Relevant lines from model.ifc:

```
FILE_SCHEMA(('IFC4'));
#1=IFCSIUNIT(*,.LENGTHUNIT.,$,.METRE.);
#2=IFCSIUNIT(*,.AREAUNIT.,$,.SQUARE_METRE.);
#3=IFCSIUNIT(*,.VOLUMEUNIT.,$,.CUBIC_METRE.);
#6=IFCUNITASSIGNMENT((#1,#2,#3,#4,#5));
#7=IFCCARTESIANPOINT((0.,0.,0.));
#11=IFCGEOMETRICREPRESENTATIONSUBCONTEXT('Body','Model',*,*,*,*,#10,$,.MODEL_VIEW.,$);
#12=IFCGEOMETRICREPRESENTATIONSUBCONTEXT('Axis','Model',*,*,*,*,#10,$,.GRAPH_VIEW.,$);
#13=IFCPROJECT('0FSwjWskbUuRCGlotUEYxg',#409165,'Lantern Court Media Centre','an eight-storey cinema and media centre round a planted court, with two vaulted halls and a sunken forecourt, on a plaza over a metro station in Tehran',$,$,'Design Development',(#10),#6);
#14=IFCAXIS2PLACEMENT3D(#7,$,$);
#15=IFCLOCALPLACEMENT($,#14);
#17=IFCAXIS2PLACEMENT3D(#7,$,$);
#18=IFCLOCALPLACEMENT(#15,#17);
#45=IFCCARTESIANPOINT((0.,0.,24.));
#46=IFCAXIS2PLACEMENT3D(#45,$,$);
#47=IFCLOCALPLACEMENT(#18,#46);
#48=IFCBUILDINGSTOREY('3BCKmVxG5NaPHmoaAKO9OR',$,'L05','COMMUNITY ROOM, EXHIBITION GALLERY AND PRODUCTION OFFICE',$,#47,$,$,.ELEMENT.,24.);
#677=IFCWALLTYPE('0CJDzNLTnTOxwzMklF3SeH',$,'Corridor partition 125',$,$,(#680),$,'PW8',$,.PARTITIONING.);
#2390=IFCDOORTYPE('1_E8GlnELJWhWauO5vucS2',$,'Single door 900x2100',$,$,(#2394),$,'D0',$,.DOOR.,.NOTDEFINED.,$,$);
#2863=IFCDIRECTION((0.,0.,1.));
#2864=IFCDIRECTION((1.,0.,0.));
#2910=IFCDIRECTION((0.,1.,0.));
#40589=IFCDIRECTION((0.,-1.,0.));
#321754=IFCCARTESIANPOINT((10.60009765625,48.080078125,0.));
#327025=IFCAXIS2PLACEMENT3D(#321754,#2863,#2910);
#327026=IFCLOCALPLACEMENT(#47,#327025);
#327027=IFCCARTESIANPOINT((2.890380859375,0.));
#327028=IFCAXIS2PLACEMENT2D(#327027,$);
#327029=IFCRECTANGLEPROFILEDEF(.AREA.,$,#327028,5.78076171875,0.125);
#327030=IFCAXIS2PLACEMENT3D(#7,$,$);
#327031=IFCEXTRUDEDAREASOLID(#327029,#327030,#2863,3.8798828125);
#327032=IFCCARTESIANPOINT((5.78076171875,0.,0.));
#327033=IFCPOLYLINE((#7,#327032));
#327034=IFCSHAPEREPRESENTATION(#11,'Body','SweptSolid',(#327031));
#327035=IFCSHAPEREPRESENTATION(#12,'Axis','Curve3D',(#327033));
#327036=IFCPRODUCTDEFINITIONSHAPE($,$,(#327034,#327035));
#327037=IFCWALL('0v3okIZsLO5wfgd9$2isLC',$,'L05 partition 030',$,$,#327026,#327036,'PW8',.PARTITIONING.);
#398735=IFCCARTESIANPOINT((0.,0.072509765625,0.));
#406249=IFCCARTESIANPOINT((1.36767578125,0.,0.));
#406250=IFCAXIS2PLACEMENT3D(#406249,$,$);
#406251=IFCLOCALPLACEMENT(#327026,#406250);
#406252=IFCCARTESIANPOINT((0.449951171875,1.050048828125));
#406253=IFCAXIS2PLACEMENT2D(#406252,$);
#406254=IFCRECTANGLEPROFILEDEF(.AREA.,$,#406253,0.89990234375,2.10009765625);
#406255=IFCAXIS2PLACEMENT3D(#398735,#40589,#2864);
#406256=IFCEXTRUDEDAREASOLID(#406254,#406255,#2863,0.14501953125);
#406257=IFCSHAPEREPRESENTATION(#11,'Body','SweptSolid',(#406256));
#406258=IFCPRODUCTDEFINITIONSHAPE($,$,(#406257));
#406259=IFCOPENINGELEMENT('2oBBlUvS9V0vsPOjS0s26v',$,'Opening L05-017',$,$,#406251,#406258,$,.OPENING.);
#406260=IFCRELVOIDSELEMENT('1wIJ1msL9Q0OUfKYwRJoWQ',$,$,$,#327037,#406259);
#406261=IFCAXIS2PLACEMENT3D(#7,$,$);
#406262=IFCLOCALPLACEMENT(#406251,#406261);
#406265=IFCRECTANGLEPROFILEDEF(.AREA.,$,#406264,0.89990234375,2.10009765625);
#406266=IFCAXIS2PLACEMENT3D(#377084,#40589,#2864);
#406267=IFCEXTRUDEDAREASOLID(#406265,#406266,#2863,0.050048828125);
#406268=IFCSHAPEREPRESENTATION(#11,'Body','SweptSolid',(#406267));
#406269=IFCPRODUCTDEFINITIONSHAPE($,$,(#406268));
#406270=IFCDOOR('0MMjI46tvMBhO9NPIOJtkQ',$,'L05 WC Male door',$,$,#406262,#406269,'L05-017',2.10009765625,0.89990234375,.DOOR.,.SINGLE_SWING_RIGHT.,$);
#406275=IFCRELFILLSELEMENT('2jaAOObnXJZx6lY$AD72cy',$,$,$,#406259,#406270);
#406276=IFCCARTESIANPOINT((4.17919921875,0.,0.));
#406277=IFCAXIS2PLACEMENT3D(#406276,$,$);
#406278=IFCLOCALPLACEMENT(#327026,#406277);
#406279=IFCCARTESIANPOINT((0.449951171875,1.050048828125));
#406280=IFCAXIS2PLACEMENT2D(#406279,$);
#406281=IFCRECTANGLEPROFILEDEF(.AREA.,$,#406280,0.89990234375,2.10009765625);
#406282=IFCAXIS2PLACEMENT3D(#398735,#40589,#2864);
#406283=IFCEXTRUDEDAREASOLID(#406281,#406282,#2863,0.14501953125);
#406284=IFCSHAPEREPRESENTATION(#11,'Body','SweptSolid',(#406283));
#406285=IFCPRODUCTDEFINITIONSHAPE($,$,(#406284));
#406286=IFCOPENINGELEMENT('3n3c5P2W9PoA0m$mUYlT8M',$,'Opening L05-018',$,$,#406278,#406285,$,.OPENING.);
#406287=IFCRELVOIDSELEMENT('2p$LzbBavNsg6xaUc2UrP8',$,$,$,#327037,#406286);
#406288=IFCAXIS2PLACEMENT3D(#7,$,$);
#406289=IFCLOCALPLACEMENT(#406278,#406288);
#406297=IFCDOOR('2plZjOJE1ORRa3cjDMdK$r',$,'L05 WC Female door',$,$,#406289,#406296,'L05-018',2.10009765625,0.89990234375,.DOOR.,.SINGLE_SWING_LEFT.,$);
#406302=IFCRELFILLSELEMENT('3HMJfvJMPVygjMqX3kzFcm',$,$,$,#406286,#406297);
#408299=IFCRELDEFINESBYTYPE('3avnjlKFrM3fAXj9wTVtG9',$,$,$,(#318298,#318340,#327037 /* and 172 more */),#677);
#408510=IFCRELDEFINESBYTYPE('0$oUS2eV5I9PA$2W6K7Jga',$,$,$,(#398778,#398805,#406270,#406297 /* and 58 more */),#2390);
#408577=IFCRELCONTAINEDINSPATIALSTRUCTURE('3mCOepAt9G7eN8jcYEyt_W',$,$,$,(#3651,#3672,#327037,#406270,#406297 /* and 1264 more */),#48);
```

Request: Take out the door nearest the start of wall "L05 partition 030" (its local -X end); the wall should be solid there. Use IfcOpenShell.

```python
import ifcopenshell
import ifcopenshell.api.feature
import ifcopenshell.api.root
import ifcopenshell.geom
import ifcopenshell.util.shape

model = ifcopenshell.open("model.ifc")
settings = ifcopenshell.geom.settings()


def volume(element):
    """Net volume in cubic metres, openings subtracted."""
    shape = ifcopenshell.geom.create_shape(settings, element)
    return ifcopenshell.util.shape.get_volume(shape.geometry)


door = model.by_guid("0MMjI46tvMBhO9NPIOJtkQ")
opening = door.FillsVoids[0].RelatingOpeningElement
wall = opening.VoidsElements[0].RelatingBuildingElement
before = volume(wall)

ifcopenshell.api.root.remove_product(model, product=door)
ifcopenshell.api.feature.remove_feature(model, feature=opening)

after = volume(wall)

print(f"wall volume {before:.3f} -> {after:.3f} m3")

model.write("model-out.ifc")
```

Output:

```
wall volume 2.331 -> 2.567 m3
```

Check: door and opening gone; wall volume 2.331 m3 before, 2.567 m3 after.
